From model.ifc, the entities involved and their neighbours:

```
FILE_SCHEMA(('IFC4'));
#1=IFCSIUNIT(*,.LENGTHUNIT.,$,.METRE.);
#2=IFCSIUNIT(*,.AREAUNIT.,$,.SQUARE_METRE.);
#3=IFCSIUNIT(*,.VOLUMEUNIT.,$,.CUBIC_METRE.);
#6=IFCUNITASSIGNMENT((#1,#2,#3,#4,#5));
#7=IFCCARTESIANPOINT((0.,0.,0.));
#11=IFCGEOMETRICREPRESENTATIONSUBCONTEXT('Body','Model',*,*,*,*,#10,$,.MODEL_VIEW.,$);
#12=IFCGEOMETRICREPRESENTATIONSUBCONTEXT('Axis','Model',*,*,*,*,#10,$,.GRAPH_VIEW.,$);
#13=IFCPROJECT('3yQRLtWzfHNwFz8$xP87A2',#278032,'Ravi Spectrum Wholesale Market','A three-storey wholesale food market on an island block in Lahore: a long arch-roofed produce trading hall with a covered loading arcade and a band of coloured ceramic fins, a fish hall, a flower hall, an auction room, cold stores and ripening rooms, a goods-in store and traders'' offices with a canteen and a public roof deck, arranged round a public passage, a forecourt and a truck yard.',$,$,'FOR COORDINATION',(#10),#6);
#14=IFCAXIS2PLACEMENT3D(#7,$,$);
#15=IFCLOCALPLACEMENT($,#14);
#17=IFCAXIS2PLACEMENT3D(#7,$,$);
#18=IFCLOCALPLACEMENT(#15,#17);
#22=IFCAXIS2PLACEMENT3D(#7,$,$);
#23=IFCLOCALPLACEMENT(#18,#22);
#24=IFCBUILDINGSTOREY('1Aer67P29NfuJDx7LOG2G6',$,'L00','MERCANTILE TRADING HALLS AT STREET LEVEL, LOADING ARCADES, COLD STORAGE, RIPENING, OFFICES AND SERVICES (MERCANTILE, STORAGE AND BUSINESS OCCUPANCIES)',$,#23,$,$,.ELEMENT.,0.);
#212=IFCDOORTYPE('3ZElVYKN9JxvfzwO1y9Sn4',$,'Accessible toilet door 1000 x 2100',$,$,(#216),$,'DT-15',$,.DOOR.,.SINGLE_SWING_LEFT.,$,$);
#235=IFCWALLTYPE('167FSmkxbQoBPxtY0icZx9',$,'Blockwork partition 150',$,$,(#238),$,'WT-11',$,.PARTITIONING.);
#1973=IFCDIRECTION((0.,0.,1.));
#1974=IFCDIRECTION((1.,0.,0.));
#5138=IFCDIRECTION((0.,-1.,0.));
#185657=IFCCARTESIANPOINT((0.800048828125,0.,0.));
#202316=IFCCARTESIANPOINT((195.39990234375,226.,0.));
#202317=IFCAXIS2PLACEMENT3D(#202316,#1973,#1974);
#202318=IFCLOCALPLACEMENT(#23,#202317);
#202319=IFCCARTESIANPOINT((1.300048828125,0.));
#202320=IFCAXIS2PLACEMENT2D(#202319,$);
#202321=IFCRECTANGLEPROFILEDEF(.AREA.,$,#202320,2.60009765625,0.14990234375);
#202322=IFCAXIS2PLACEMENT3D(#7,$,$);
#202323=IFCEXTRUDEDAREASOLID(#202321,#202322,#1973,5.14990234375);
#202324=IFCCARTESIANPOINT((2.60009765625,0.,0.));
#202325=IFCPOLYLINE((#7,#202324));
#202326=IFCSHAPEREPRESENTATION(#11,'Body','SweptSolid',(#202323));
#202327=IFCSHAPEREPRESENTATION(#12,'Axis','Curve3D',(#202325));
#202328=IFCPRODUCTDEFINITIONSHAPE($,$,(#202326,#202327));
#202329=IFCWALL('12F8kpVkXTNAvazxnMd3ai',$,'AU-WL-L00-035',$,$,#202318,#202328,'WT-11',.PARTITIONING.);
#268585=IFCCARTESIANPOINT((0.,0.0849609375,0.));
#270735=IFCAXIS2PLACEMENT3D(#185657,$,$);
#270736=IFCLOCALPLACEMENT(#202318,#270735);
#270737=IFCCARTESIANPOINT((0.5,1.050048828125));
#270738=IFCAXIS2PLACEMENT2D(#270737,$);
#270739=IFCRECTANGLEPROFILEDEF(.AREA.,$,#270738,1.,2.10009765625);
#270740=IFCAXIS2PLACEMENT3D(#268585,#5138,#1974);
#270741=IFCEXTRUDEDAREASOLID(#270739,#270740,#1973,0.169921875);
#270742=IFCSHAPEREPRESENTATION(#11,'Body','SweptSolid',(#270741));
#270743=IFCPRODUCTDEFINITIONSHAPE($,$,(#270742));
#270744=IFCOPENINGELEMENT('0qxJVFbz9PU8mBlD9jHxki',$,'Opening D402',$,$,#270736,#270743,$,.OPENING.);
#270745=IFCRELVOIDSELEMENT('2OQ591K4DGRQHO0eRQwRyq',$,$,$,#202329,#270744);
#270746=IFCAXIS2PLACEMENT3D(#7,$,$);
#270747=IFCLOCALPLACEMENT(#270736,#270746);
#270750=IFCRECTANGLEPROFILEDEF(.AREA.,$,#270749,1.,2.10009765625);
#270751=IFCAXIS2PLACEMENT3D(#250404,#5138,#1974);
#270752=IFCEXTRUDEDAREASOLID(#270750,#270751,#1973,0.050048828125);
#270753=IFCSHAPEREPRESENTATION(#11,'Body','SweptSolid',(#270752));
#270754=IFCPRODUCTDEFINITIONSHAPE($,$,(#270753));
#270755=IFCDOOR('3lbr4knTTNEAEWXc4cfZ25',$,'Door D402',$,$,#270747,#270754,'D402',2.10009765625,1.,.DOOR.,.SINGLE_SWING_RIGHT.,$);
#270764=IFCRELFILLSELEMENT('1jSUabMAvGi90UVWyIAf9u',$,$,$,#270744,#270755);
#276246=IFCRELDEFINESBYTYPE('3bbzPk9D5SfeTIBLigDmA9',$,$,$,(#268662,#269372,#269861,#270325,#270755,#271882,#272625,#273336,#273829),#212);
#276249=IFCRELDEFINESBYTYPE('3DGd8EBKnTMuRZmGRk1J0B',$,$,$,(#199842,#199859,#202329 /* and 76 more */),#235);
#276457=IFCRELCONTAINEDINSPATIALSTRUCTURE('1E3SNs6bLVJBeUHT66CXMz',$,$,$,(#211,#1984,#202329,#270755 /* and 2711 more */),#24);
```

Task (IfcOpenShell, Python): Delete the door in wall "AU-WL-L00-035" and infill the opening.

```python
import ifcopenshell
import ifcopenshell.api.feature
import ifcopenshell.api.root
import ifcopenshell.geom
import ifcopenshell.util.shape

model = ifcopenshell.open("model.ifc")
settings = ifcopenshell.geom.settings()


def volume(element):
    """Net volume in cubic metres, openings subtracted."""
    shape = ifcopenshell.geom.create_shape(settings, element)
    return ifcopenshell.util.shape.get_volume(shape.geometry)


door = model.by_id(270755)
opening = door.FillsVoids[0].RelatingOpeningElement
wall = opening.VoidsElements[0].RelatingBuildingElement
before = volume(wall)

ifcopenshell.api.root.remove_product(model, product=door)
ifcopenshell.api.feature.remove_feature(model, feature=opening)

after = volume(wall)

print(f"wall volume {before:.3f} -> {after:.3f} m3")

model.write("model_v2.ifc")
```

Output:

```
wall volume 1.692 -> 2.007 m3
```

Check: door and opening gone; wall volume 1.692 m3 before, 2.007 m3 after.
